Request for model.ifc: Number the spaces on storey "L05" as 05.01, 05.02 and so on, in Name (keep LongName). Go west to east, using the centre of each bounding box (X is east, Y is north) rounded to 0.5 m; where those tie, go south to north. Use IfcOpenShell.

First a look at what the model holds.

```python
import ifcopenshell
import ifcopenshell.util.element
import ifcopenshell.util.placement

model = ifcopenshell.open("model.ifc")
print(model.schema)
storey = next(s for s in model.by_type("IfcBuildingStorey") if s.Name == "L05")
spaces = [e for e in ifcopenshell.util.element.get_decomposition(storey) if e.is_a("IfcSpace")]
for e in sorted(spaces, key=lambda e: e.id()):
    origin = ifcopenshell.util.placement.get_local_placement(e.ObjectPlacement)[:3, 3]
    print(e.id(), e.Name, e.LongName, origin.round(2) + 0.0, sep=" | ")
```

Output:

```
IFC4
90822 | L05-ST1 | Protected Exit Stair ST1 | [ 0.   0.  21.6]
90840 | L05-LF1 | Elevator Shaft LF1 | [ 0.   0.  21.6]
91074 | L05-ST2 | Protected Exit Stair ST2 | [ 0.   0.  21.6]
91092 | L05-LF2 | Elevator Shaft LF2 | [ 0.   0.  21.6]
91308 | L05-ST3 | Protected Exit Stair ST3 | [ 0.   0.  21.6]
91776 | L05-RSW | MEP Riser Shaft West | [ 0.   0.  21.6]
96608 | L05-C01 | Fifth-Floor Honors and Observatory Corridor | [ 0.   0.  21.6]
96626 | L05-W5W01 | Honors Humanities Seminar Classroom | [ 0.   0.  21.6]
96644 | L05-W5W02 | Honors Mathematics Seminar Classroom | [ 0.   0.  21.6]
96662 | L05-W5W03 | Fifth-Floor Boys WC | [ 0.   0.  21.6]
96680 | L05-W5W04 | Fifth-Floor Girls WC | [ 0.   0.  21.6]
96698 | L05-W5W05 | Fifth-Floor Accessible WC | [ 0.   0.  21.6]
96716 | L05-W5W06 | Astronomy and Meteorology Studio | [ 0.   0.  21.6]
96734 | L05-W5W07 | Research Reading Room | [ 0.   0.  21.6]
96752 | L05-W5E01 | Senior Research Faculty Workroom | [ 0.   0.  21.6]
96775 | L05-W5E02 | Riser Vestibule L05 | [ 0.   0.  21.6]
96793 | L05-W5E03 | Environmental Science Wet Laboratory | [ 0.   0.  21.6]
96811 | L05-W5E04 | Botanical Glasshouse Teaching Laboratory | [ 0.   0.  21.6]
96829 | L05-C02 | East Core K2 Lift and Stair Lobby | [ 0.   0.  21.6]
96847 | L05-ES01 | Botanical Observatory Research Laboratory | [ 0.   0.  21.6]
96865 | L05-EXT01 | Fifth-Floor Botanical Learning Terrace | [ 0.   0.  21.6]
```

```python
import ifcopenshell
import ifcopenshell.geom
import ifcopenshell.util.element
import ifcopenshell.util.shape

model = ifcopenshell.open("model.ifc")
settings = ifcopenshell.geom.settings()
settings.set("use-world-coords", True)


def centre(element):
    shape = ifcopenshell.geom.create_shape(settings, element)
    return ifcopenshell.util.shape.get_bbox_centroid(shape.geometry)


storey = next(s for s in model.by_type("IfcBuildingStorey") if s.Name == "L05")
spaces = [e for e in ifcopenshell.util.element.get_decomposition(storey) if e.is_a("IfcSpace")]

# Insertion points can sit at a corner or the storey origin, so sort by the geometry (in metres).
centres = {e: centre(e) for e in spaces}
spaces.sort(key=lambda e: (round(centres[e][0] / 0.5), centres[e][1]))

for i, e in enumerate(spaces, start=1):
    number = f"05.{i:02d}"
    e.Name = number
    print(e.id(), number)

model.write("model_v2.ifc")
```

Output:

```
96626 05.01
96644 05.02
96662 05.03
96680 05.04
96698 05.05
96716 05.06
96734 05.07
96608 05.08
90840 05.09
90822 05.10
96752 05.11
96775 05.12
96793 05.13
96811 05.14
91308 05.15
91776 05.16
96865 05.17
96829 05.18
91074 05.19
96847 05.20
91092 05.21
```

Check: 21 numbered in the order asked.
